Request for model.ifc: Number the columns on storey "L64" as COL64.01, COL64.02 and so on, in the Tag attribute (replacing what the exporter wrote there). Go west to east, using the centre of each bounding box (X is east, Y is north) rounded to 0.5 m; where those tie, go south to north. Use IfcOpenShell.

First a look at what the model holds.

```python
import ifcopenshell
import ifcopenshell.util.element
import ifcopenshell.util.placement

model = ifcopenshell.open("model.ifc")
print(model.schema)
storey = next(s for s in model.by_type("IfcBuildingStorey") if s.Name == "L64")
columns = [e for e in ifcopenshell.util.element.get_decomposition(storey) if e.is_a("IfcColumn")]
for e in sorted(columns, key=lambda e: e.id()):
    origin = ifcopenshell.util.placement.get_local_placement(e.ObjectPlacement)[:3, 3]
    print(e.id(), e.Tag, e.Name, origin.round(2) + 0.0, sep=" | ")
```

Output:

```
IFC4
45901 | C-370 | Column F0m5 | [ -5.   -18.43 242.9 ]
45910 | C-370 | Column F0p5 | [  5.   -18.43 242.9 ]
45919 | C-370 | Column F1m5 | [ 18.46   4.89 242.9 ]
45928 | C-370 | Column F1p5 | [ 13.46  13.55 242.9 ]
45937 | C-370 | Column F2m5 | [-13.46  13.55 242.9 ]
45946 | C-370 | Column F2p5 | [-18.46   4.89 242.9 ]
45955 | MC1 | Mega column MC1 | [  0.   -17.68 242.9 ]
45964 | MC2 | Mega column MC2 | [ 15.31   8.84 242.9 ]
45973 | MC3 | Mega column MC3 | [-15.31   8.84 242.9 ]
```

```python
import ifcopenshell
import ifcopenshell.geom
import ifcopenshell.util.element
import ifcopenshell.util.shape

model = ifcopenshell.open("model.ifc")
settings = ifcopenshell.geom.settings()
settings.set("use-world-coords", True)


def centre(element):
    shape = ifcopenshell.geom.create_shape(settings, element)
    return ifcopenshell.util.shape.get_bbox_centroid(shape.geometry)


storey = next(s for s in model.by_type("IfcBuildingStorey") if s.Name == "L64")
columns = [e for e in ifcopenshell.util.element.get_decomposition(storey) if e.is_a("IfcColumn")]

# Insertion points can sit at a corner or the storey origin, so sort by the geometry (in metres).
centres = {e: centre(e) for e in columns}
columns.sort(key=lambda e: (round(centres[e][0] / 0.5), centres[e][1]))

for i, e in enumerate(columns, start=1):
    number = f"COL64.{i:02d}"
    e.Tag = number
    print(e.id(), number)

model.write("model_v2.ifc")
```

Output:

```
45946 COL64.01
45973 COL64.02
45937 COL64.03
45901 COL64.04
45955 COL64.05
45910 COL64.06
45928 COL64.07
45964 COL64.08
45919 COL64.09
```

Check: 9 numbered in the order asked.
